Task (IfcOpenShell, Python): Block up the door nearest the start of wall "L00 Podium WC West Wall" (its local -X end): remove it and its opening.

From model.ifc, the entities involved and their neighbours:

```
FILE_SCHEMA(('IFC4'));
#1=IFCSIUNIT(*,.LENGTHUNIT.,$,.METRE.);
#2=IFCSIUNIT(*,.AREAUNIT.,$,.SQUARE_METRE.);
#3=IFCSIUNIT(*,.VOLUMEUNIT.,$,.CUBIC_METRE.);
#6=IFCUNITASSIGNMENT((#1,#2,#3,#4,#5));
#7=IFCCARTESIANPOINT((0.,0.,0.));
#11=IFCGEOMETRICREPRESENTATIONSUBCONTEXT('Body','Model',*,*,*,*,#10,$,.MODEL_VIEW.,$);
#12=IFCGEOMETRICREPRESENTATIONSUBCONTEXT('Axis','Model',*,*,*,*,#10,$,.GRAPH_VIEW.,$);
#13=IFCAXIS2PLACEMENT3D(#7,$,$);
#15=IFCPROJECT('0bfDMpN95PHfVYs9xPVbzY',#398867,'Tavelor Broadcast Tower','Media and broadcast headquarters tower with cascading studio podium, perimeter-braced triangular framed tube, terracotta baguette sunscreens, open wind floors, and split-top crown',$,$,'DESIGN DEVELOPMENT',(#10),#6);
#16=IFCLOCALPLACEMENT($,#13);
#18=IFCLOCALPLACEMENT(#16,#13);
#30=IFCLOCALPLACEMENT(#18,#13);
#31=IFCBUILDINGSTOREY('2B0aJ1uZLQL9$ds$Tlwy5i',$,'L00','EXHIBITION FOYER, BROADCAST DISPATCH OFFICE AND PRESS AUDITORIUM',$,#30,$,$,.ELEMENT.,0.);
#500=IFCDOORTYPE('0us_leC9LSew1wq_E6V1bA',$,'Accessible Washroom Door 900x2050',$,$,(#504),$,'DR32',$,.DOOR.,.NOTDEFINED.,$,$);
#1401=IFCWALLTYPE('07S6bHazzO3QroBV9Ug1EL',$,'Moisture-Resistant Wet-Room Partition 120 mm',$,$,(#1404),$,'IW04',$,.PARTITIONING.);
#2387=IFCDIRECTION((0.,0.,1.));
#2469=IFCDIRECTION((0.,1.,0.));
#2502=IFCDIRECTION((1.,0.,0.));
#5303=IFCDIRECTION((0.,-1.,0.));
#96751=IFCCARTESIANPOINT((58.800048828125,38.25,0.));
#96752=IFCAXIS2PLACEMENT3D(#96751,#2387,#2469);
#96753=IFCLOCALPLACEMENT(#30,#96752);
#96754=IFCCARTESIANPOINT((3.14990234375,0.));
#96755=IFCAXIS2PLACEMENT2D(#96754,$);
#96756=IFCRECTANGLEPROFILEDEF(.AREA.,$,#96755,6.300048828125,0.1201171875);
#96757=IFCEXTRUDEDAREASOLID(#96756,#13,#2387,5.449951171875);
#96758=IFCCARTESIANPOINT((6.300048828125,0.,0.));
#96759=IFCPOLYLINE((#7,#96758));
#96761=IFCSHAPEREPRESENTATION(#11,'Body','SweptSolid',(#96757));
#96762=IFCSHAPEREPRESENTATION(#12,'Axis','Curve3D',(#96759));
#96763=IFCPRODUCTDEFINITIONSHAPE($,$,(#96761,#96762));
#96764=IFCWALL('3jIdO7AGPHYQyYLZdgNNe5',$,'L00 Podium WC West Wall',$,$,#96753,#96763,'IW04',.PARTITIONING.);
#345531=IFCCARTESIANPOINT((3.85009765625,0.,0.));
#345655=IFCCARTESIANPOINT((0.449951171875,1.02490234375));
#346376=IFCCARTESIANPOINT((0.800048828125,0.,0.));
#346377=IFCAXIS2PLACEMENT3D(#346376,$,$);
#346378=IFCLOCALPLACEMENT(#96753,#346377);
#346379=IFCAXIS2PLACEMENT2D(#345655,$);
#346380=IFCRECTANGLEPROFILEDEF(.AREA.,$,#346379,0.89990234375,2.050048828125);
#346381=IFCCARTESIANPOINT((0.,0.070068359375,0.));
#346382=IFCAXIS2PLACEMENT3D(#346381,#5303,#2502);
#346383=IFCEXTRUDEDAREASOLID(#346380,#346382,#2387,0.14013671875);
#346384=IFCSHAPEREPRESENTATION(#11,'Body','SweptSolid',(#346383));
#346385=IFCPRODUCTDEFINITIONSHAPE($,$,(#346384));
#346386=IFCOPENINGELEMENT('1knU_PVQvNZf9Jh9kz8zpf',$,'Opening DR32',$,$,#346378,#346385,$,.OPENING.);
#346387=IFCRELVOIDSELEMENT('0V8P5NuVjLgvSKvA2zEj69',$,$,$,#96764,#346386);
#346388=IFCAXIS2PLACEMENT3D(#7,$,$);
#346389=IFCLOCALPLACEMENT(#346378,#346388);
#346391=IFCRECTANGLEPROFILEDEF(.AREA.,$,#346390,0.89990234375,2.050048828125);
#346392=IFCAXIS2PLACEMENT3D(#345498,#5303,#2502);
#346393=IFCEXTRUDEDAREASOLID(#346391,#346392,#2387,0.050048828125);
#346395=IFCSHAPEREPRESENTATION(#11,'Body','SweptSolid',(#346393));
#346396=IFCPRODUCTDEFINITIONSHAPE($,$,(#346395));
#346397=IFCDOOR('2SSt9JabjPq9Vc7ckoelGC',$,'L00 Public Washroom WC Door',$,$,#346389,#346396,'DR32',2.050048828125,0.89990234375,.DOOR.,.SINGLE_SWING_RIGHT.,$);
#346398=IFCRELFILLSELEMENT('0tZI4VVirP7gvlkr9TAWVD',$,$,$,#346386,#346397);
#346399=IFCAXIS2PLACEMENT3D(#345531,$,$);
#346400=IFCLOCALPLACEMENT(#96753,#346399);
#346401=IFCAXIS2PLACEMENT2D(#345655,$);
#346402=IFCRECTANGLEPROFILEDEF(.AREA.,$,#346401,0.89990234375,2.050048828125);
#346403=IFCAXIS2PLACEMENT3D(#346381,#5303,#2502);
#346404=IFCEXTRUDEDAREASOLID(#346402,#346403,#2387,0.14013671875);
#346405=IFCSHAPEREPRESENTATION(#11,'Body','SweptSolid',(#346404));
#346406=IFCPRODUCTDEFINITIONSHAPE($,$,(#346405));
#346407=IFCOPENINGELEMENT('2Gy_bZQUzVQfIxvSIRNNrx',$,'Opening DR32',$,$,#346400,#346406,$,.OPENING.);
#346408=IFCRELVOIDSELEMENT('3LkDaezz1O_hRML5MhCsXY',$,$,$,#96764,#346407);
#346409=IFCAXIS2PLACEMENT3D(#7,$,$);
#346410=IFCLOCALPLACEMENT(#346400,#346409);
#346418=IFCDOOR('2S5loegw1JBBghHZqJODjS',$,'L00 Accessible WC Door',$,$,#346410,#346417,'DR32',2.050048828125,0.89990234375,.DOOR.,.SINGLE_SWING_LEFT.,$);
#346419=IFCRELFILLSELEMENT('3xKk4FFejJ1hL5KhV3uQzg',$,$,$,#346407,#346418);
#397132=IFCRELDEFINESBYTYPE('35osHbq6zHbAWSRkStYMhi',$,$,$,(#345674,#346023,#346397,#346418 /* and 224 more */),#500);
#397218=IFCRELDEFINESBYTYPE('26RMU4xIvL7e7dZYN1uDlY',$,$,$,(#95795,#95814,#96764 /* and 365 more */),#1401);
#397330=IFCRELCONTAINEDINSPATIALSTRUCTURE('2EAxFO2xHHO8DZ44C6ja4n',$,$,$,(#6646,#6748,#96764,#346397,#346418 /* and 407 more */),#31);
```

```python
import ifcopenshell
import ifcopenshell.api.feature
import ifcopenshell.api.root
import ifcopenshell.geom
import ifcopenshell.util.shape

model = ifcopenshell.open("model.ifc")
settings = ifcopenshell.geom.settings()


def volume(element):
    """Net volume in cubic metres, openings subtracted."""
    shape = ifcopenshell.geom.create_shape(settings, element)
    return ifcopenshell.util.shape.get_volume(shape.geometry)


door = model.by_guid("2SSt9JabjPq9Vc7ckoelGC")
opening = door.FillsVoids[0].RelatingOpeningElement
wall = opening.VoidsElements[0].RelatingBuildingElement
before = volume(wall)

ifcopenshell.api.root.remove_product(model, product=door)
ifcopenshell.api.feature.remove_feature(model, feature=opening)

after = volume(wall)

print(f"wall volume {before:.3f} -> {after:.3f} m3")

model.write("model_v2.ifc")
```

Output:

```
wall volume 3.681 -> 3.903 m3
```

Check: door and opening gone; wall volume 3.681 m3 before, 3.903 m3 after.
